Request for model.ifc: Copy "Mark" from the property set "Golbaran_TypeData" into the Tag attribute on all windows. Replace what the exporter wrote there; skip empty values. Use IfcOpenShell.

First a look at what the model holds.

```python
import ifcopenshell
import ifcopenshell.util.element

model = ifcopenshell.open("model.ifc")
print(model.schema)
windows = model.by_type("IfcWindow")
print(len(windows), "windows")
for e in windows[:8]:
    source = ifcopenshell.util.element.get_pset(e, "Golbaran_TypeData", "Mark")
    target = e.Tag
    print(e.id(), repr(source), repr(target), sep=" | ")
```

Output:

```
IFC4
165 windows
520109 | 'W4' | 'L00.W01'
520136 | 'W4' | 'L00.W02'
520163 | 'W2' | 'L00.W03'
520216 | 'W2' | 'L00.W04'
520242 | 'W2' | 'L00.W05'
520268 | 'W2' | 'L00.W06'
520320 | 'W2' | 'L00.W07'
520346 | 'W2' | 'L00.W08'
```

```python
import ifcopenshell
import ifcopenshell.util.element

model = ifcopenshell.open("model.ifc")

count = 0
for e in model.by_type("IfcWindow"):
    value = ifcopenshell.util.element.get_pset(e, "Golbaran_TypeData", "Mark")
    current = e.Tag
    if not value or not value.strip() or current == value:
        continue
    e.Tag = value
    count += 1

print(count, "windows updated")

model.write("model_updated.ifc")
```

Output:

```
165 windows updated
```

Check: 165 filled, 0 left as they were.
